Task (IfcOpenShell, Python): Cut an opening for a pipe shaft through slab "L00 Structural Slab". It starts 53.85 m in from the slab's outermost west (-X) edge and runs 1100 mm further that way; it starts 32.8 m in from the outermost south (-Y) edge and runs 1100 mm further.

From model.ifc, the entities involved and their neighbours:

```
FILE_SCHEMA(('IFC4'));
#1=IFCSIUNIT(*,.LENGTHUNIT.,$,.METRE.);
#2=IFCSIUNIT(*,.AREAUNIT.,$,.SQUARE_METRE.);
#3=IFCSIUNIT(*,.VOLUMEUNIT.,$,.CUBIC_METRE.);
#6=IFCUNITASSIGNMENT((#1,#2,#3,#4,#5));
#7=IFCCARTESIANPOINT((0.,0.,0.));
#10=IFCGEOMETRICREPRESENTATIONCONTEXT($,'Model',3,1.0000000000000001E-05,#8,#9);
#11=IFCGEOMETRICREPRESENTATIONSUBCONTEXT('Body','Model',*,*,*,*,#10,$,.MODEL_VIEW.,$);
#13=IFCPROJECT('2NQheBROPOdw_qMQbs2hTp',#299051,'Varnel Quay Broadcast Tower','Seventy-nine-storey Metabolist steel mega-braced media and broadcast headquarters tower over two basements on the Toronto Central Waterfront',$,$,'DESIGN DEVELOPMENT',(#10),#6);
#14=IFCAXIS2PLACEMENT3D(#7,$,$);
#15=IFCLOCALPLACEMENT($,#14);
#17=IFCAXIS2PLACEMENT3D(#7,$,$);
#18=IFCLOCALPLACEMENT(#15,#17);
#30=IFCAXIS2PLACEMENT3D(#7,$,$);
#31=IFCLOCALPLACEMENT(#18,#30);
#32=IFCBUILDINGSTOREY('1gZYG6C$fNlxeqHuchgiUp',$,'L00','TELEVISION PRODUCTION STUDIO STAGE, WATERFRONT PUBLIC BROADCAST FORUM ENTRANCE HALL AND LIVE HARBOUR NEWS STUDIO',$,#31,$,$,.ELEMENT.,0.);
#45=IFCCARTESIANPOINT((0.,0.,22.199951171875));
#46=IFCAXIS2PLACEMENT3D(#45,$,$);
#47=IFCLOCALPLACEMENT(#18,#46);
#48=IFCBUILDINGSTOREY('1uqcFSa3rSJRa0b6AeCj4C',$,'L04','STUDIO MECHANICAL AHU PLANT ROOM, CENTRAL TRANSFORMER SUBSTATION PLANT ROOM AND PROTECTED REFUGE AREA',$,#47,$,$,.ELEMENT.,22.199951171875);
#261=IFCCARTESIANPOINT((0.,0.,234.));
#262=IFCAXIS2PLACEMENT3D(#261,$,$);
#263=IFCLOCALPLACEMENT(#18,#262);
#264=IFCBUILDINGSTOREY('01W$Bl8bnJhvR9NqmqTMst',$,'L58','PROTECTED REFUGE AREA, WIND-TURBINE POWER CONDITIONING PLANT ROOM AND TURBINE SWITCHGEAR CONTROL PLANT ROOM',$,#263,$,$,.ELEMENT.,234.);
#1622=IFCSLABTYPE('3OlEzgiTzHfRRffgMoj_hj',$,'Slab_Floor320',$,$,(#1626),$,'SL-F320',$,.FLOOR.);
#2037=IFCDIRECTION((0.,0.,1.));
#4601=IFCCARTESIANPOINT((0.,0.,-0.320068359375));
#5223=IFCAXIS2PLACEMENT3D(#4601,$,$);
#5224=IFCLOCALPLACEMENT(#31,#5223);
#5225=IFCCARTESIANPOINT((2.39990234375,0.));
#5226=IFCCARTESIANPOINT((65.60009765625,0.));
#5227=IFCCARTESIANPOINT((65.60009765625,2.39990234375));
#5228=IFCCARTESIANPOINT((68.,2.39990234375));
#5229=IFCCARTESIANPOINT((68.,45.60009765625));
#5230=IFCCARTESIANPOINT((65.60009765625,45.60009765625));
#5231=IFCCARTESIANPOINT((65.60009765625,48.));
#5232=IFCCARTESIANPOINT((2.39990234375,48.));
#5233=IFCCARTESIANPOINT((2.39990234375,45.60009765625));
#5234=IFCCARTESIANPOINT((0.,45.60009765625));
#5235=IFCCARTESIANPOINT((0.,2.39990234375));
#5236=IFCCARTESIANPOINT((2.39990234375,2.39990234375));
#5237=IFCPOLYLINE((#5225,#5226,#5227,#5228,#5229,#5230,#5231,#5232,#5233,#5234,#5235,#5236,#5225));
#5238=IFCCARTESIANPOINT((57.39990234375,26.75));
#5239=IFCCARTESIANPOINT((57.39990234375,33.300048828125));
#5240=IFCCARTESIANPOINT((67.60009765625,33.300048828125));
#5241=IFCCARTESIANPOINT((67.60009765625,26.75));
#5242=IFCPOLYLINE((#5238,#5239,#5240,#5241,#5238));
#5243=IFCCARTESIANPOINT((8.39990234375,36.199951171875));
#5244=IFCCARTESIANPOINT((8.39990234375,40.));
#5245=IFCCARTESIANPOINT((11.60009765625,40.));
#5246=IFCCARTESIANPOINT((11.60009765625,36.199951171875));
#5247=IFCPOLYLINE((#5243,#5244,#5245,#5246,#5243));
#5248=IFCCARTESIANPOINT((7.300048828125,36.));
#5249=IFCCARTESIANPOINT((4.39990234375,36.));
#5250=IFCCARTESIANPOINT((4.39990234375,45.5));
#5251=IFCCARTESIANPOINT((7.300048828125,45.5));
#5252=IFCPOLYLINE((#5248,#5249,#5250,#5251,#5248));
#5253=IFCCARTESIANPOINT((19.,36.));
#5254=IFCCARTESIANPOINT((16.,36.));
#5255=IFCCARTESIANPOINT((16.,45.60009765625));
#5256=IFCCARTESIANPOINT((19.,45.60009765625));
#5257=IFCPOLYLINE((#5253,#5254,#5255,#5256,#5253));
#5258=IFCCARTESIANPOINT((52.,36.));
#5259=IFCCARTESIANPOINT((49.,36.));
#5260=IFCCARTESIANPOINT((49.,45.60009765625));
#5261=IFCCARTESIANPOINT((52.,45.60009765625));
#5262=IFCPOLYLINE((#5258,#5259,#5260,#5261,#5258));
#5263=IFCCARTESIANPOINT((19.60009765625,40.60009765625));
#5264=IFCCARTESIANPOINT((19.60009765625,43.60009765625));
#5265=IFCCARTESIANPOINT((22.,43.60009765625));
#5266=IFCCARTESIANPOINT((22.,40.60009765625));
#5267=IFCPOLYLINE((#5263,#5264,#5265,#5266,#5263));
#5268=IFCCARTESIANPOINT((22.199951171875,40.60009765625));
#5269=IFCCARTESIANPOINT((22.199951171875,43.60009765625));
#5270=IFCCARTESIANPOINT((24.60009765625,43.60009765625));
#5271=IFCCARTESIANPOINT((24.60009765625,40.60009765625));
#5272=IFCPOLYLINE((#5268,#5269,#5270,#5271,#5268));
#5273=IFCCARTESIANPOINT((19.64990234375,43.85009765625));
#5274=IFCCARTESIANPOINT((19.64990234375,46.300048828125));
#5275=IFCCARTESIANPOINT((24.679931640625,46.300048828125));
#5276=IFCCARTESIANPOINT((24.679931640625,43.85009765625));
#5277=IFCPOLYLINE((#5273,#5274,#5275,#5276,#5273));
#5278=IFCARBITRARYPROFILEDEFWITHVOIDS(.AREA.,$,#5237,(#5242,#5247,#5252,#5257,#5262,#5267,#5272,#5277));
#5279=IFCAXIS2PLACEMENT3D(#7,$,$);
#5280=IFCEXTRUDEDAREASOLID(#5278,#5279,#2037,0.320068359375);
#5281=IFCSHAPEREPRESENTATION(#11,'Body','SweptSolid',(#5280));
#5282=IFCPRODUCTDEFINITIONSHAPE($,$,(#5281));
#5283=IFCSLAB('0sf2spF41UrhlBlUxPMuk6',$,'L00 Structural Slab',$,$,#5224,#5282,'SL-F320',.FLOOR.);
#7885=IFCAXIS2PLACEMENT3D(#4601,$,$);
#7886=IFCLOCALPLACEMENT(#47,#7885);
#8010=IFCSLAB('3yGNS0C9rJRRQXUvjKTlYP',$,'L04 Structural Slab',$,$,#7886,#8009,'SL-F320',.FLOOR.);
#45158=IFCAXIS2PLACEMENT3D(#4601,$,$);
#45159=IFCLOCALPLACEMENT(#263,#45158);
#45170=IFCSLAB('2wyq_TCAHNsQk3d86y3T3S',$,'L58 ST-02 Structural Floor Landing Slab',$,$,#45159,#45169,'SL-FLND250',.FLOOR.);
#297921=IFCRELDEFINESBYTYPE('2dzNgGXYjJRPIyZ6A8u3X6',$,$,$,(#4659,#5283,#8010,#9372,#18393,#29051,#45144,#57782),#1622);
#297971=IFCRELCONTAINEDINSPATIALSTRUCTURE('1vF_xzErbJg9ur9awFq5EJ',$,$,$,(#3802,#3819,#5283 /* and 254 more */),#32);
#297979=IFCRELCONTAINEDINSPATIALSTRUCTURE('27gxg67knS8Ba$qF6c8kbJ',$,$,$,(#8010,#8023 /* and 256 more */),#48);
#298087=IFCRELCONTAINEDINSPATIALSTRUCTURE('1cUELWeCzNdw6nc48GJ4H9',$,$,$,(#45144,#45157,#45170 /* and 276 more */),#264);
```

```python
import numpy as np
import ifcopenshell
import ifcopenshell.api.feature
import ifcopenshell.api.geometry
import ifcopenshell.api.root
import ifcopenshell.geom
import ifcopenshell.util.placement
import ifcopenshell.util.representation
import ifcopenshell.util.shape
import ifcopenshell.util.unit

model = ifcopenshell.open("model.ifc")
unit_scale = ifcopenshell.util.unit.calculate_unit_scale(model)
settings = ifcopenshell.geom.settings()


def volume(element):
    """Net volume in cubic metres, openings subtracted."""
    shape = ifcopenshell.geom.create_shape(settings, element)
    return ifcopenshell.util.shape.get_volume(shape.geometry)


slab = model.by_id(5283)
before = volume(slab)

# Extent in the slab's own axes, in metres. The edges named are its -X and -Y sides.
slab_shape = ifcopenshell.geom.create_shape(settings, slab)
vertices = ifcopenshell.util.shape.get_vertices(slab_shape.geometry)
x_min, y_min, bottom = vertices.min(axis=0)
top = vertices[:, 2].max()

opening = ifcopenshell.api.root.create_entity(model, ifc_class="IfcOpeningElement", name="Pipe shaft opening", predefined_type="OPENING")
context = ifcopenshell.util.representation.get_context(model, "Model", "Body", "MODEL_VIEW")
width, depth = 1.1, 1.1
outline = [(0.0, 0.0), (width, 0.0), (width, depth), (0.0, depth), (0.0, 0.0)]
# Overshoot both faces by 50 mm so the cut is clean.
shape = ifcopenshell.api.geometry.add_slab_representation(
    model, context=context, depth=top - bottom + 0.1, polyline=outline
)
ifcopenshell.api.geometry.assign_representation(model, product=opening, representation=shape)

matrix = ifcopenshell.util.placement.get_local_placement(slab.ObjectPlacement)
matrix[:, 3] = matrix @ np.append(np.array([x_min + 53.85, y_min + 32.8, bottom - 0.05]) / unit_scale, 1.0)
ifcopenshell.api.geometry.edit_object_placement(model, product=opening, matrix=matrix, is_si=False)
ifcopenshell.api.feature.add_feature(model, feature=opening, element=slab)

after = volume(slab)

print(f"slab volume {before:.3f} -> {after:.3f} m3")

model.write("model_edited.ifc")
```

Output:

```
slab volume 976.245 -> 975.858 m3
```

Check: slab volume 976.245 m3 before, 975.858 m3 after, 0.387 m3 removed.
